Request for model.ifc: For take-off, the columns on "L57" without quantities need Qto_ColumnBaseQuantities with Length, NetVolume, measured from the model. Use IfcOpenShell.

First a look at what the model holds.

```python
import ifcopenshell
import ifcopenshell.util.element
import ifcopenshell.util.unit

model = ifcopenshell.open("model.ifc")
print(model.schema)
for unit_type in ("LENGTHUNIT", "AREAUNIT", "VOLUMEUNIT"):
    print(unit_type, ifcopenshell.util.unit.calculate_unit_scale(model, unit_type))
storey = next(s for s in model.by_type("IfcBuildingStorey") if s.Name == "L57")
columns = [e for e in ifcopenshell.util.element.get_decomposition(storey) if e.is_a("IfcColumn")]
for e in sorted(columns, key=lambda e: e.id()):
    print(e.id(), e.is_a(), e.Name, list(ifcopenshell.util.element.get_psets(e, qtos_only=True)), sep=" | ")
```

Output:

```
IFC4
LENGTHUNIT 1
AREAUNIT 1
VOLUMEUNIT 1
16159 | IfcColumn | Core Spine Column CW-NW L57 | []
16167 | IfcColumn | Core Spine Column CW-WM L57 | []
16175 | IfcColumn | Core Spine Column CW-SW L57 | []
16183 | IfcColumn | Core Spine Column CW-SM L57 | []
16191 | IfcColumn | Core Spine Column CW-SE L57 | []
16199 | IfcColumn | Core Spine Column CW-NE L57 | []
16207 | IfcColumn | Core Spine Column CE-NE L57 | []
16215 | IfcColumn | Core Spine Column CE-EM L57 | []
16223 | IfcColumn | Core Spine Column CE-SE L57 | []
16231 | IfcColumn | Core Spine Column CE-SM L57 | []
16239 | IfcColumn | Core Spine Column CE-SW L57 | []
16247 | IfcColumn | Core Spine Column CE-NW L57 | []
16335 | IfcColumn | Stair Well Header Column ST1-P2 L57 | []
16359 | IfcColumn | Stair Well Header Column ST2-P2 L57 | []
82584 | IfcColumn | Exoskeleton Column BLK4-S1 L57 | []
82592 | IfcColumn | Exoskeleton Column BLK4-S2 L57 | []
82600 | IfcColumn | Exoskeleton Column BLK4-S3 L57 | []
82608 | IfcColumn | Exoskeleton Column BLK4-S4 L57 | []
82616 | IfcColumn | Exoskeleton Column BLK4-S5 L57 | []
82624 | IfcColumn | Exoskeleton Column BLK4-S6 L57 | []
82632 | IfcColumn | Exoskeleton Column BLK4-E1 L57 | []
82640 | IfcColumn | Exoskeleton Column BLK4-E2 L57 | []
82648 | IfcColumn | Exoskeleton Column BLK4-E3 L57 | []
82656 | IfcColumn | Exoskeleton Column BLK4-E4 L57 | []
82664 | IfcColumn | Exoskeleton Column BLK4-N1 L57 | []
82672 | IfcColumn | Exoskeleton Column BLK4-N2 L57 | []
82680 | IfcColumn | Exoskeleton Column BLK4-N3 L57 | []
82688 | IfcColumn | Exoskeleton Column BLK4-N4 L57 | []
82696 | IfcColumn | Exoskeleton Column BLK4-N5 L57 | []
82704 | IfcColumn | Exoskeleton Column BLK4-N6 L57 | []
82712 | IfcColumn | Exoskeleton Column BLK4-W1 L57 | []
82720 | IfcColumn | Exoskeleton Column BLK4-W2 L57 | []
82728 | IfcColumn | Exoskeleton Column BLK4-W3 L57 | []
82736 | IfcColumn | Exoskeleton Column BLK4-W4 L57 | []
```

```python
import ifcopenshell
import ifcopenshell.api.pset
import ifcopenshell.geom
import ifcopenshell.util.element
import ifcopenshell.util.shape
import ifcopenshell.util.unit

model = ifcopenshell.open("model.ifc")
unit_scale = ifcopenshell.util.unit.calculate_unit_scale(model)
volume_scale = ifcopenshell.util.unit.calculate_unit_scale(model, "VOLUMEUNIT")
settings = ifcopenshell.geom.settings()

storey = next(s for s in model.by_type("IfcBuildingStorey") if s.Name == "L57")
columns = [e for e in ifcopenshell.util.element.get_decomposition(storey) if e.is_a("IfcColumn")]

for e in sorted(columns, key=lambda e: e.id()):
    if ifcopenshell.util.element.get_psets(e, qtos_only=True, should_inherit=False):
        continue
    # Geometry comes back in metres, in the element's own axes.
    shape = ifcopenshell.geom.create_shape(settings, e)
    values = {
        "Length": ifcopenshell.util.shape.get_z(shape.geometry) / unit_scale,
        "NetVolume": ifcopenshell.util.shape.get_volume(shape.geometry) / volume_scale,
    }
    qto = ifcopenshell.api.pset.add_qto(model, product=e, name="Qto_ColumnBaseQuantities")
    ifcopenshell.api.pset.edit_qto(model, qto=qto, properties=values)
    print(e.id(), {k: round(v, 3) for k, v in values.items()})

model.write("model_v2.ifc")
```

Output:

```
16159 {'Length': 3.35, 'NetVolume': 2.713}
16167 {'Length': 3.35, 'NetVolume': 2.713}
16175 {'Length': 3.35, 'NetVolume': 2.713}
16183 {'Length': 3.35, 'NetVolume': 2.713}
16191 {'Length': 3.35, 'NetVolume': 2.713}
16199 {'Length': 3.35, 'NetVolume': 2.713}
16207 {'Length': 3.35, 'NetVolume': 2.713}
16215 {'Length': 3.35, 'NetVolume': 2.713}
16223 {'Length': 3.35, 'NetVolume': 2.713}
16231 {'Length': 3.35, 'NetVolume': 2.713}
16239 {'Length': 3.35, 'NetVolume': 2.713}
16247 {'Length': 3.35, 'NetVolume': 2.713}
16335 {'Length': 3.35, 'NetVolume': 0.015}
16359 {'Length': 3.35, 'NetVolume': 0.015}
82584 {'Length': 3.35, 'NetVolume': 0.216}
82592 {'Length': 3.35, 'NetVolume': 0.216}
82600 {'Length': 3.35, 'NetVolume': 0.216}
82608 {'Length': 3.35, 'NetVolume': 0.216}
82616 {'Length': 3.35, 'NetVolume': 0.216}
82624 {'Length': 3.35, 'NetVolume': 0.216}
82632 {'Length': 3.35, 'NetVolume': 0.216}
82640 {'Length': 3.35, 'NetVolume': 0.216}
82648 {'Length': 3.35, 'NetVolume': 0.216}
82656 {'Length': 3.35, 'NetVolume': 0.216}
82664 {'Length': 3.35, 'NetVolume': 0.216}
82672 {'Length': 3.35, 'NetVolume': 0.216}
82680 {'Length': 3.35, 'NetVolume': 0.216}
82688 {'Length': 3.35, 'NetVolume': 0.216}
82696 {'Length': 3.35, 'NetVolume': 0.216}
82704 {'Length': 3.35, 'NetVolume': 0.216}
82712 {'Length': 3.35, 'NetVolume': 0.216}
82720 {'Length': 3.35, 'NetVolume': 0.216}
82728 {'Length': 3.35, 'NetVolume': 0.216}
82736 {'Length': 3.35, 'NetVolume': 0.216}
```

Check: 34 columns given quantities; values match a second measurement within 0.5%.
